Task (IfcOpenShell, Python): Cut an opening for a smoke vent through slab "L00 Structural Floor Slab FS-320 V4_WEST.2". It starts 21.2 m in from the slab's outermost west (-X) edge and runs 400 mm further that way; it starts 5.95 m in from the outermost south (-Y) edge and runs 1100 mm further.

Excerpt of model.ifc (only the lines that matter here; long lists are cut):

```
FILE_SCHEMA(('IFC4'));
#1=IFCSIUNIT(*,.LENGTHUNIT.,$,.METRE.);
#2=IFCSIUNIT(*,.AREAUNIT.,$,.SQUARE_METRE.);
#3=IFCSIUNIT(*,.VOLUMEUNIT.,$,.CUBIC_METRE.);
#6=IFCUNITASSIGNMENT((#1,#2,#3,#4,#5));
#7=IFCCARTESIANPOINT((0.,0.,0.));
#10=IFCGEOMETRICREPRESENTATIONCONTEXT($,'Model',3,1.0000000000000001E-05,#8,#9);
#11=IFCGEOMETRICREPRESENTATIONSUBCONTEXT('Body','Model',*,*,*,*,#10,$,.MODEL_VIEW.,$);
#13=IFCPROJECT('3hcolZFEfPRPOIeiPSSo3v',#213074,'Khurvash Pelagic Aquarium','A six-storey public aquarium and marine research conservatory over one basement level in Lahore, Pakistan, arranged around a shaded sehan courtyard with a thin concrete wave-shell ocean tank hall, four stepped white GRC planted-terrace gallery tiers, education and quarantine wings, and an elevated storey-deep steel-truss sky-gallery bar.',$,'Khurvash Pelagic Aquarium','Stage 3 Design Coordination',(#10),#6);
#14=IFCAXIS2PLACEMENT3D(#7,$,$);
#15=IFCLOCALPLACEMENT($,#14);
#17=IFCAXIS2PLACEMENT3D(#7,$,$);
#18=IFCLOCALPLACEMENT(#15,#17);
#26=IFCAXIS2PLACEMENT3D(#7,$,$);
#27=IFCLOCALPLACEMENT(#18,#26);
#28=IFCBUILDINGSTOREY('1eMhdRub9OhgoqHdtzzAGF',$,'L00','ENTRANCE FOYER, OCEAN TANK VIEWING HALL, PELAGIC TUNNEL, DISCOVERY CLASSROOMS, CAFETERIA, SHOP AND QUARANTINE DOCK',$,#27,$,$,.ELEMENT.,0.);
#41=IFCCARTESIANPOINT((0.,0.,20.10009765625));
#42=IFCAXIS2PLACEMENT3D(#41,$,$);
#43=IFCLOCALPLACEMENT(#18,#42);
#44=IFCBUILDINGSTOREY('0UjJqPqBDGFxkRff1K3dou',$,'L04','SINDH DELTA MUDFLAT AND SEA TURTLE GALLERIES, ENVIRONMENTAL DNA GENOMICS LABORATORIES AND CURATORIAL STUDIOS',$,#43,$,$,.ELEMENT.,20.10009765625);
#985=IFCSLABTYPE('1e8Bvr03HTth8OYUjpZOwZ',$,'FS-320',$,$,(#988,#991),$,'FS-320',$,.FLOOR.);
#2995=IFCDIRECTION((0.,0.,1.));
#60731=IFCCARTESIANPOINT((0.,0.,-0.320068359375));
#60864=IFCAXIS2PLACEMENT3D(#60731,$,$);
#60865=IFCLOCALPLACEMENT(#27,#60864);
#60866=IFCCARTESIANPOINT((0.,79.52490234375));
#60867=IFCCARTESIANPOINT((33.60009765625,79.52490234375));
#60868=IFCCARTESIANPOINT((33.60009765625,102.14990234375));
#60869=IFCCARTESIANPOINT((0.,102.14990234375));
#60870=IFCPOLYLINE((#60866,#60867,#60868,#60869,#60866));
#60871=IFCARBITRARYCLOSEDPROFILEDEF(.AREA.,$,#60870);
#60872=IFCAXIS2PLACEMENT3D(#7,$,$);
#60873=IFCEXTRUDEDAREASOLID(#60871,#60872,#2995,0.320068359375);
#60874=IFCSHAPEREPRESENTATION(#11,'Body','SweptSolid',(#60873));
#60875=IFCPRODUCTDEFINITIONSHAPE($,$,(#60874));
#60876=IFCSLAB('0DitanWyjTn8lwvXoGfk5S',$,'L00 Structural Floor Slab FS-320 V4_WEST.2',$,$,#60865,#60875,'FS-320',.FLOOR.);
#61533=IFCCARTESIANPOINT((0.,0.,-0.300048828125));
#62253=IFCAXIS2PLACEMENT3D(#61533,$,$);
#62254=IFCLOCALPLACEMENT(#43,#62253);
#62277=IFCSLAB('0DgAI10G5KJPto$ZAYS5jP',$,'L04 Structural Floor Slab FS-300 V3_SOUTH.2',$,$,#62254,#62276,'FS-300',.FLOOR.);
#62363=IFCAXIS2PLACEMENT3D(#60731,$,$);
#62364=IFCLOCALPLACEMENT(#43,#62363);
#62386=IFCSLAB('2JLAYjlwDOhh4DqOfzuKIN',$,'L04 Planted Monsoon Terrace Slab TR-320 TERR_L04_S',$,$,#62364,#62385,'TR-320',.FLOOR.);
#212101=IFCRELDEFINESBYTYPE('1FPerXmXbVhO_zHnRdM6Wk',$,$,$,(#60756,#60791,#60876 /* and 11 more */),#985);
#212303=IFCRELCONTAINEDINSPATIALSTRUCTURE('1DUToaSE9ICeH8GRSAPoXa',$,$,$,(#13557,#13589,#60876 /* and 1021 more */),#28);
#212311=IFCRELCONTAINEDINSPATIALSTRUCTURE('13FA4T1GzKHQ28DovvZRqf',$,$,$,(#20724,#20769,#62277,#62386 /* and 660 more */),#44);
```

```python
import numpy as np
import ifcopenshell
import ifcopenshell.api.feature
import ifcopenshell.api.geometry
import ifcopenshell.api.root
import ifcopenshell.geom
import ifcopenshell.util.placement
import ifcopenshell.util.representation
import ifcopenshell.util.shape
import ifcopenshell.util.unit

model = ifcopenshell.open("model.ifc")
unit_scale = ifcopenshell.util.unit.calculate_unit_scale(model)
settings = ifcopenshell.geom.settings()


def volume(element):
    """Net volume in cubic metres, openings subtracted."""
    shape = ifcopenshell.geom.create_shape(settings, element)
    return ifcopenshell.util.shape.get_volume(shape.geometry)


slab = model.by_id(60876)
before = volume(slab)

# Extent in the slab's own axes, in metres. The edges named are its -X and -Y sides.
slab_shape = ifcopenshell.geom.create_shape(settings, slab)
vertices = ifcopenshell.util.shape.get_vertices(slab_shape.geometry)
x_min, y_min, bottom = vertices.min(axis=0)
top = vertices[:, 2].max()

opening = ifcopenshell.api.root.create_entity(model, ifc_class="IfcOpeningElement", name="Smoke vent opening", predefined_type="OPENING")
context = ifcopenshell.util.representation.get_context(model, "Model", "Body", "MODEL_VIEW")
width, depth = 0.4, 1.1
outline = [(0.0, 0.0), (width, 0.0), (width, depth), (0.0, depth), (0.0, 0.0)]
# Overshoot both faces by 50 mm so the cut is clean.
shape = ifcopenshell.api.geometry.add_slab_representation(
    model, context=context, depth=top - bottom + 0.1, polyline=outline
)
ifcopenshell.api.geometry.assign_representation(model, product=opening, representation=shape)

matrix = ifcopenshell.util.placement.get_local_placement(slab.ObjectPlacement)
matrix[:, 3] = matrix @ np.append(np.array([x_min + 21.2, y_min + 5.95, bottom - 0.05]) / unit_scale, 1.0)
ifcopenshell.api.geometry.edit_object_placement(model, product=opening, matrix=matrix, is_si=False)
ifcopenshell.api.feature.add_feature(model, feature=opening, element=slab)

after = volume(slab)

print(f"slab volume {before:.3f} -> {after:.3f} m3")

model.write("model_rev.ifc")
```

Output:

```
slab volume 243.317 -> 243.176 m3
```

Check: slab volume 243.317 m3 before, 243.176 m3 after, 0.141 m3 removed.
